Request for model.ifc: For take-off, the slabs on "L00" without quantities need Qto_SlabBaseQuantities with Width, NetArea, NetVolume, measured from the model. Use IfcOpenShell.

First a look at what the model holds.

```python
import ifcopenshell
import ifcopenshell.util.element
import ifcopenshell.util.unit

model = ifcopenshell.open("model.ifc")
print(model.schema)
for unit_type in ("LENGTHUNIT", "AREAUNIT", "VOLUMEUNIT"):
    print(unit_type, ifcopenshell.util.unit.calculate_unit_scale(model, unit_type))
storey = next(s for s in model.by_type("IfcBuildingStorey") if s.Name == "L00")
slabs = [e for e in ifcopenshell.util.element.get_decomposition(storey) if e.is_a("IfcSlab")]
for e in sorted(slabs, key=lambda e: e.id()):
    print(e.id(), e.is_a(), e.Name, list(ifcopenshell.util.element.get_psets(e, qtos_only=True)), sep=" | ")
```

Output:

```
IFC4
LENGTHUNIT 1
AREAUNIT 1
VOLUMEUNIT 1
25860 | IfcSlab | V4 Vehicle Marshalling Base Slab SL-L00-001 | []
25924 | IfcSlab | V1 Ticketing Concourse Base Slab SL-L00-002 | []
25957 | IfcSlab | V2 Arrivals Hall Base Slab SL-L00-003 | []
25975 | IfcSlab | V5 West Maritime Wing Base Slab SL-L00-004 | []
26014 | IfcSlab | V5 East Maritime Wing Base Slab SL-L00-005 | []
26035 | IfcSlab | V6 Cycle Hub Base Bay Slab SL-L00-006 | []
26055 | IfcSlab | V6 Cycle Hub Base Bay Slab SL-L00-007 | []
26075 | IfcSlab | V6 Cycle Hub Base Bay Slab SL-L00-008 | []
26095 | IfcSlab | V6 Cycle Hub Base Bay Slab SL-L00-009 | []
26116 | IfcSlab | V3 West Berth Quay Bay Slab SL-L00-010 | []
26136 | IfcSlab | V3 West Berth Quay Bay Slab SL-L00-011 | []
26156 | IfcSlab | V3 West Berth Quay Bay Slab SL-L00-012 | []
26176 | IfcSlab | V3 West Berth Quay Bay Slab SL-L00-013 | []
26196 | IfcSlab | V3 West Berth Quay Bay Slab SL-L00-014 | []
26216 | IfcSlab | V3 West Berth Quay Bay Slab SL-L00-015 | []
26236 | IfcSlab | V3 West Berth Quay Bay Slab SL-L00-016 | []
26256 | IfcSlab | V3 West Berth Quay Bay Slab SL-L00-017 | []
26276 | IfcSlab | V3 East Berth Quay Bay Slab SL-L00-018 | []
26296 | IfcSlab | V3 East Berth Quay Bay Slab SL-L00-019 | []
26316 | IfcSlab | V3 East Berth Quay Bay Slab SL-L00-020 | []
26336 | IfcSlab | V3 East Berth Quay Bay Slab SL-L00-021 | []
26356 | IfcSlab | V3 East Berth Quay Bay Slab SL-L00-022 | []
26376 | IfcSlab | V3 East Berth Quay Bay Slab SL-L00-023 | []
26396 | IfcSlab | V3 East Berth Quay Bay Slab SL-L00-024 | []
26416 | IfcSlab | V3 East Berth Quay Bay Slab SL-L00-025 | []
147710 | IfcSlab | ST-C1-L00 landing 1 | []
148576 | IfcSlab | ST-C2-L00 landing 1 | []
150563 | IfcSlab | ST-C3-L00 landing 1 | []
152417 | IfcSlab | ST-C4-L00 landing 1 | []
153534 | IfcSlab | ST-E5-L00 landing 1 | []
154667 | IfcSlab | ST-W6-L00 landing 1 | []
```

```python
import ifcopenshell
import ifcopenshell.api.pset
import ifcopenshell.geom
import ifcopenshell.util.element
import ifcopenshell.util.shape
import ifcopenshell.util.unit

model = ifcopenshell.open("model.ifc")
unit_scale = ifcopenshell.util.unit.calculate_unit_scale(model)
area_scale = ifcopenshell.util.unit.calculate_unit_scale(model, "AREAUNIT")
volume_scale = ifcopenshell.util.unit.calculate_unit_scale(model, "VOLUMEUNIT")
settings = ifcopenshell.geom.settings()

storey = next(s for s in model.by_type("IfcBuildingStorey") if s.Name == "L00")
slabs = [e for e in ifcopenshell.util.element.get_decomposition(storey) if e.is_a("IfcSlab")]

for e in sorted(slabs, key=lambda e: e.id()):
    if ifcopenshell.util.element.get_psets(e, qtos_only=True, should_inherit=False):
        continue
    # Geometry comes back in metres, in the element's own axes.
    shape = ifcopenshell.geom.create_shape(settings, e)
    values = {
        "Width": ifcopenshell.util.shape.get_z(shape.geometry) / unit_scale,
        "NetArea": ifcopenshell.util.shape.get_footprint_area(shape.geometry) / area_scale,
        "NetVolume": ifcopenshell.util.shape.get_volume(shape.geometry) / volume_scale,
    }
    qto = ifcopenshell.api.pset.add_qto(model, product=e, name="Qto_SlabBaseQuantities")
    ifcopenshell.api.pset.edit_qto(model, qto=qto, properties=values)
    print(e.id(), {k: round(v, 3) for k, v in values.items()})

model.write("model_updated.ifc")
```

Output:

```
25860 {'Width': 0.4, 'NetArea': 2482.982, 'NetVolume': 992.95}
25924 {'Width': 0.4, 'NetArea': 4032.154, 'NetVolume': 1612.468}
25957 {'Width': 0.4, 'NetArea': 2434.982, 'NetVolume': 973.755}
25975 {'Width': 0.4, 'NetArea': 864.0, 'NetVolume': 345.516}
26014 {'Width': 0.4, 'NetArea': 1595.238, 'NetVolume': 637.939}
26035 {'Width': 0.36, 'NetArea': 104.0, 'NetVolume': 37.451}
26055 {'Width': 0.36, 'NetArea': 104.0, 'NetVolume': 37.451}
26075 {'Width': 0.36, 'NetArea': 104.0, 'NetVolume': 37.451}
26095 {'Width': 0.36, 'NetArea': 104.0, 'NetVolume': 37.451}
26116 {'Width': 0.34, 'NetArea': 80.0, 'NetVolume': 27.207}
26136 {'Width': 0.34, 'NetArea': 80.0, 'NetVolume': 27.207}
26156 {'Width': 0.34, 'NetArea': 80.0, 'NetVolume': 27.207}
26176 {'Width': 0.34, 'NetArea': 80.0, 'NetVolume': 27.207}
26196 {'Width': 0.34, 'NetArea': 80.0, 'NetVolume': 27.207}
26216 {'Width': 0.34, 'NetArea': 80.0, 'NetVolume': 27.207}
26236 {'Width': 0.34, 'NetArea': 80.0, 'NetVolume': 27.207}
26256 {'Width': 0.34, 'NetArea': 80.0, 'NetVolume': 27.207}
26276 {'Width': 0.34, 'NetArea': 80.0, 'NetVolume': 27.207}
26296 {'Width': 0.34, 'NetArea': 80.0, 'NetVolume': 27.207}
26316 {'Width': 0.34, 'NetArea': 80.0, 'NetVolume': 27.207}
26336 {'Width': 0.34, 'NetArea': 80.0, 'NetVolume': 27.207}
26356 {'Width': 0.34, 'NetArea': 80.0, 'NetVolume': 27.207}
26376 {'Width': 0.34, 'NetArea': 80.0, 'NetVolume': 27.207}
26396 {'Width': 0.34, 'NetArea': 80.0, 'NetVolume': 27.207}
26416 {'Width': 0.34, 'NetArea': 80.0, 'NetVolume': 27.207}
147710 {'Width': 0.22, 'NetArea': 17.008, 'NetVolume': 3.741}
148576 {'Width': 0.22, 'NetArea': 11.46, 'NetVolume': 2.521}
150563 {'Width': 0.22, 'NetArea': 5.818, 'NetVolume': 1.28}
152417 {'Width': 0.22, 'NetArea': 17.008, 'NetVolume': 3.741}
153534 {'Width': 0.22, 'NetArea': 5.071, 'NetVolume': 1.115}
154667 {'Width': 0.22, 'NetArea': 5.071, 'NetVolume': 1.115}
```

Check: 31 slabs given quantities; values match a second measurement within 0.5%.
